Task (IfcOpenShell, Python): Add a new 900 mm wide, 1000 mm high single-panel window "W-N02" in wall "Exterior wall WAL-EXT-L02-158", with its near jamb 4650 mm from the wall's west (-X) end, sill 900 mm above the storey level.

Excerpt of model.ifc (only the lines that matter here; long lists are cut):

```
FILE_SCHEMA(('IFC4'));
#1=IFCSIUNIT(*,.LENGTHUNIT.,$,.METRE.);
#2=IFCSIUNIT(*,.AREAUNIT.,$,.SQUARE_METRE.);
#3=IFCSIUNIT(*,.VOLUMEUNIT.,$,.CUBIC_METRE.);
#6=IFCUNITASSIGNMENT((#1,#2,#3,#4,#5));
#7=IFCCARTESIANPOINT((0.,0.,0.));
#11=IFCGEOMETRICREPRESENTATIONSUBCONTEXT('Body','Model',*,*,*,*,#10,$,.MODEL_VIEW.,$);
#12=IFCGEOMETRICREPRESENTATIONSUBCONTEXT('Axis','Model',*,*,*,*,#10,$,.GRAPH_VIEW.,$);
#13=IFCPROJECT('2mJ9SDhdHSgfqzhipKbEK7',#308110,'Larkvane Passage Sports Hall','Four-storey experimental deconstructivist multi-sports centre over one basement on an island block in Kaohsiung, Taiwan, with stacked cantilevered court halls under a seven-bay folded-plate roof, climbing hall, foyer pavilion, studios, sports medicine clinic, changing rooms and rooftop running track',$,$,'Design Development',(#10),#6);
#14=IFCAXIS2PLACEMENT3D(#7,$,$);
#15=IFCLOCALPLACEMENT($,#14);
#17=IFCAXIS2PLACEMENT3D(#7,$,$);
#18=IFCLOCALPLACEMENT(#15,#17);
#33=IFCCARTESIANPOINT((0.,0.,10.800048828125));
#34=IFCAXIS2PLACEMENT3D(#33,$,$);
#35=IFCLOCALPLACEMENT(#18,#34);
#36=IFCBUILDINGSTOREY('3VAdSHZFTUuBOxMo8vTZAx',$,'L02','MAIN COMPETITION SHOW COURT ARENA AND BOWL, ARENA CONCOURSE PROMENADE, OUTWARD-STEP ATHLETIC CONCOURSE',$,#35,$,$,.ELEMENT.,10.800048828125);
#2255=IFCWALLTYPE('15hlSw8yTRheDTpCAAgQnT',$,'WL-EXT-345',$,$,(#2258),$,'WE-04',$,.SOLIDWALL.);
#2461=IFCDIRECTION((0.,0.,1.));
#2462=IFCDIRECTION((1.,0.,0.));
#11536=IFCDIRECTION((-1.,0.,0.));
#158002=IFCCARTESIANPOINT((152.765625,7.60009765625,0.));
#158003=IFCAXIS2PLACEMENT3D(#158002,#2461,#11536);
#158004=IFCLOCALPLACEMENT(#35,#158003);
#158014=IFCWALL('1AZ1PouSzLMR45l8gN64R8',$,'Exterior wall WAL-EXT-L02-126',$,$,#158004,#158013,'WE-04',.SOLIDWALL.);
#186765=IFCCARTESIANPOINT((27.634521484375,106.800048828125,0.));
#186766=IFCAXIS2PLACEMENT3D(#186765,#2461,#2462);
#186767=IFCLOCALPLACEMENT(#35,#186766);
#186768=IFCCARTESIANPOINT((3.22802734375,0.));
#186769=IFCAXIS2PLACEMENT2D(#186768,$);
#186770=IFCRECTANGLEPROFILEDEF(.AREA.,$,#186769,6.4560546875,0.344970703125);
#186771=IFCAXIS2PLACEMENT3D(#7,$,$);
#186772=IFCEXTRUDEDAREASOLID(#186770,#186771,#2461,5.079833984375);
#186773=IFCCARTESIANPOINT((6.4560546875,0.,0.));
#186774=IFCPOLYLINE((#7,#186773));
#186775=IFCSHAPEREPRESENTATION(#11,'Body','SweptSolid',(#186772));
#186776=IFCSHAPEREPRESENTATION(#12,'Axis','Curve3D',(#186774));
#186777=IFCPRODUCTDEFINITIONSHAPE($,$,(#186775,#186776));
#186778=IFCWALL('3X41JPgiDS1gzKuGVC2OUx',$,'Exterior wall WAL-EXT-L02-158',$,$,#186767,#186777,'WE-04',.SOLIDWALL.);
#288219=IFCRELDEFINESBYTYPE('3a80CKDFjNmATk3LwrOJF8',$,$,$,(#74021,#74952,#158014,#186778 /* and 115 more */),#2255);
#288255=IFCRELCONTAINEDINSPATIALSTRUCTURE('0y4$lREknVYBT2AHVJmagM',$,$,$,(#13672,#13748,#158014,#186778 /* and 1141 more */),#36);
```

```python
import numpy as np
import ifcopenshell
import ifcopenshell.api.feature
import ifcopenshell.api.geometry
import ifcopenshell.api.root
import ifcopenshell.api.spatial
import ifcopenshell.geom
import ifcopenshell.util.element
import ifcopenshell.util.placement
import ifcopenshell.util.representation
import ifcopenshell.util.shape
import ifcopenshell.util.unit

model = ifcopenshell.open("model.ifc")
unit_scale = ifcopenshell.util.unit.calculate_unit_scale(model)
settings = ifcopenshell.geom.settings()


def volume(element):
    """Net volume in cubic metres, openings subtracted."""
    shape = ifcopenshell.geom.create_shape(settings, element)
    return ifcopenshell.util.shape.get_volume(shape.geometry)


wall = model.by_guid("3X41JPgiDS1gzKuGVC2OUx")
storey = ifcopenshell.util.element.get_container(wall, ifc_class="IfcBuildingStorey")
context = ifcopenshell.util.representation.get_context(model, "Model", "Body", "MODEL_VIEW")
before = volume(wall)

width, height, from_end, sill = 0.9, 1, 4.65, 0.9  # metres

# The wall runs along its own X axis, and the end named is its -X end.
wall_shape = ifcopenshell.geom.create_shape(settings, wall)
x, y, z = ifcopenshell.util.shape.get_vertices(wall_shape.geometry).T
start = x.min() + from_end
face, thickness = float(y.min()), float(y.max() - y.min())
wall_matrix = ifcopenshell.util.placement.get_local_placement(wall.ObjectPlacement)
level = ifcopenshell.util.placement.get_local_placement(storey.ObjectPlacement)[2, 3]


def in_wall(x, y):
    """Placement at x, y metres in the wall's axes, at sill height."""
    matrix = wall_matrix.copy()
    matrix[:, 3] = wall_matrix @ np.array([x / unit_scale, y / unit_scale, 0.0, 1.0])
    matrix[2, 3] = level + sill / unit_scale
    return matrix


# Opening: a box that overshoots both wall faces by 50 mm.
opening = ifcopenshell.api.root.create_entity(model, ifc_class="IfcOpeningElement", predefined_type="OPENING")
box = ifcopenshell.api.geometry.add_wall_representation(
    model, context=context, length=width, height=height, thickness=thickness + 0.1
)
ifcopenshell.api.geometry.assign_representation(model, product=opening, representation=box)
ifcopenshell.api.geometry.edit_object_placement(model, product=opening, matrix=in_wall(start, face - 0.05), is_si=False)
ifcopenshell.api.feature.add_feature(model, feature=opening, element=wall)

window = ifcopenshell.api.root.create_entity(model, ifc_class="IfcWindow", name="W-N02", predefined_type="WINDOW")
window.OverallWidth, window.OverallHeight = width / unit_scale, height / unit_scale
window.PartitioningType = "SINGLE_PANEL"
body = ifcopenshell.api.geometry.add_window_representation(
    model,
    context=context,
    overall_width=window.OverallWidth,
    overall_height=window.OverallHeight,
    partition_type="SINGLE_PANEL",
)
ifcopenshell.api.geometry.assign_representation(model, product=window, representation=body)
ifcopenshell.api.spatial.assign_container(model, products=[window], relating_structure=storey)
ifcopenshell.api.feature.add_filling(model, opening=opening, element=window)

# Centre the window in the wall's thickness.
ifcopenshell.api.geometry.edit_object_placement(model, product=window, matrix=in_wall(start, face), is_si=False)
window_shape = ifcopenshell.geom.create_shape(settings, window)
depth = ifcopenshell.util.shape.get_vertices(window_shape.geometry)[:, 1]
offset = face + thickness / 2 - (depth.min() + depth.max()) / 2
ifcopenshell.api.geometry.edit_object_placement(model, product=window, matrix=in_wall(start, offset), is_si=False)

after = volume(wall)

print(f"wall volume {before:.3f} -> {after:.3f} m3")

model.write("model_v2.ifc")
```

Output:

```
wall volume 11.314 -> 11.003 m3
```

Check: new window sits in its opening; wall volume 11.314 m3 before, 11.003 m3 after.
